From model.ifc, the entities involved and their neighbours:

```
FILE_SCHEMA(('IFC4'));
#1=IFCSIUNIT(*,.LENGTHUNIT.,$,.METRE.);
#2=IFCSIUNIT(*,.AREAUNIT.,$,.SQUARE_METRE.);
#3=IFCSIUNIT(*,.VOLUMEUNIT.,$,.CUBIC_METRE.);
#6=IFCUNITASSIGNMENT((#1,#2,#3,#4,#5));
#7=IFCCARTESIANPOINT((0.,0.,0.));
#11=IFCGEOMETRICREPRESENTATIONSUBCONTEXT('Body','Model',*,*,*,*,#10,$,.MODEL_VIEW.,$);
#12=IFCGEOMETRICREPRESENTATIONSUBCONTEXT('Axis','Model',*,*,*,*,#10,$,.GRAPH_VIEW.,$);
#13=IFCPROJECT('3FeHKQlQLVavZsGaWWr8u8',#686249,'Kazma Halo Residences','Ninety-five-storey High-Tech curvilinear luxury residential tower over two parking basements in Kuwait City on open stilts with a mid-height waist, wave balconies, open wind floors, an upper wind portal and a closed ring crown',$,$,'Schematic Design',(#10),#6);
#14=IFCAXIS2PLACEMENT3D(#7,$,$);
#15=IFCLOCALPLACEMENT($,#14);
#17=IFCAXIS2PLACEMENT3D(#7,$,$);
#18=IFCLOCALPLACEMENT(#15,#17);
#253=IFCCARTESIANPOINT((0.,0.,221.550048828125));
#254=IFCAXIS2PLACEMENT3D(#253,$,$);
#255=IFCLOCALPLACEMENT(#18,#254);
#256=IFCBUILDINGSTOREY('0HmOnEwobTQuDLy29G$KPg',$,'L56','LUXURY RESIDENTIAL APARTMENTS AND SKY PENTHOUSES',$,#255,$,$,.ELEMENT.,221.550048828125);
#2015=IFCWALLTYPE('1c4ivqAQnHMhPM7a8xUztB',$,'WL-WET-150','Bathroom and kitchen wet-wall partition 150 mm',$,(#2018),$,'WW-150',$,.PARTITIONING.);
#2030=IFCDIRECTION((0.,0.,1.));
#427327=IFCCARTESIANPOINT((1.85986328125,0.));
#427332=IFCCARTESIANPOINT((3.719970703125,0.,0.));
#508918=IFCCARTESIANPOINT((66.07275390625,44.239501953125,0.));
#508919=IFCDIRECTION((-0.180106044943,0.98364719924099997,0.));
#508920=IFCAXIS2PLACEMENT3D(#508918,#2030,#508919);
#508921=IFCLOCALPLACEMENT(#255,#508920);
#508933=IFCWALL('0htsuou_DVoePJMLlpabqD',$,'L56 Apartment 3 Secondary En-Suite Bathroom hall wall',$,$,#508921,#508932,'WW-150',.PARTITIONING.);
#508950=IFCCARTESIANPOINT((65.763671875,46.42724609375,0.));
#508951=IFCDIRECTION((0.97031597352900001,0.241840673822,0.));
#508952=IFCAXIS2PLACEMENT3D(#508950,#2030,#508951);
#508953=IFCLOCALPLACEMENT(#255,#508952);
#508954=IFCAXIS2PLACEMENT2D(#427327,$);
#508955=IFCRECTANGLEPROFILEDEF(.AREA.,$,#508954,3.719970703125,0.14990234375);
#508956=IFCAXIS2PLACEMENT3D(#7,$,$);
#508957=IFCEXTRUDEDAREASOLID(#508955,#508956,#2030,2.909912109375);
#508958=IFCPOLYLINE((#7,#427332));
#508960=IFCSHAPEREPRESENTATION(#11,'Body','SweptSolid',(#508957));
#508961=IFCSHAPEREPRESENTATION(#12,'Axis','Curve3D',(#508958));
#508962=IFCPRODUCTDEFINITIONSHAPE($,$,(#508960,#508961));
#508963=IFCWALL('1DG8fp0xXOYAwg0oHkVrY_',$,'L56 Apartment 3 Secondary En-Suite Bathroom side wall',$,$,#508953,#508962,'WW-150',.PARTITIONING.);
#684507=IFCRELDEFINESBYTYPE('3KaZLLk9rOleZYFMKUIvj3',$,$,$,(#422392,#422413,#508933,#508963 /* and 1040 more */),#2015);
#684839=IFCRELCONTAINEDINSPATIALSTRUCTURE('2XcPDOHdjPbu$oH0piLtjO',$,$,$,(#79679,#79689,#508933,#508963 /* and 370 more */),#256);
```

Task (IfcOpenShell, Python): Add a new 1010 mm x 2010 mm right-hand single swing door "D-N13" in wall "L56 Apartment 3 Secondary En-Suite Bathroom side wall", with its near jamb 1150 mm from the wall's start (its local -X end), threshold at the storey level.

```python
import numpy as np
import ifcopenshell
import ifcopenshell.api.feature
import ifcopenshell.api.geometry
import ifcopenshell.api.root
import ifcopenshell.api.spatial
import ifcopenshell.geom
import ifcopenshell.util.element
import ifcopenshell.util.placement
import ifcopenshell.util.representation
import ifcopenshell.util.shape
import ifcopenshell.util.unit

model = ifcopenshell.open("model.ifc")
unit_scale = ifcopenshell.util.unit.calculate_unit_scale(model)
settings = ifcopenshell.geom.settings()


def volume(element):
    """Net volume in cubic metres, openings subtracted."""
    shape = ifcopenshell.geom.create_shape(settings, element)
    return ifcopenshell.util.shape.get_volume(shape.geometry)


wall = model.by_id(508963)
storey = ifcopenshell.util.element.get_container(wall, ifc_class="IfcBuildingStorey")
context = ifcopenshell.util.representation.get_context(model, "Model", "Body", "MODEL_VIEW")
before = volume(wall)

width, height, from_end, sill = 1.01, 2.01, 1.15, 0.0  # metres

# The wall runs along its own X axis, and the end named is its -X end.
wall_shape = ifcopenshell.geom.create_shape(settings, wall)
x, y, z = ifcopenshell.util.shape.get_vertices(wall_shape.geometry).T
start = x.min() + from_end
face, thickness = float(y.min()), float(y.max() - y.min())
wall_matrix = ifcopenshell.util.placement.get_local_placement(wall.ObjectPlacement)
level = ifcopenshell.util.placement.get_local_placement(storey.ObjectPlacement)[2, 3]


def in_wall(x, y):
    """Placement at x, y metres in the wall's axes, at sill height."""
    matrix = wall_matrix.copy()
    matrix[:, 3] = wall_matrix @ np.array([x / unit_scale, y / unit_scale, 0.0, 1.0])
    matrix[2, 3] = level + sill / unit_scale
    return matrix


# Opening: a box that overshoots both wall faces by 50 mm.
opening = ifcopenshell.api.root.create_entity(model, ifc_class="IfcOpeningElement", predefined_type="OPENING")
box = ifcopenshell.api.geometry.add_wall_representation(
    model, context=context, length=width, height=height, thickness=thickness + 0.1
)
ifcopenshell.api.geometry.assign_representation(model, product=opening, representation=box)
ifcopenshell.api.geometry.edit_object_placement(model, product=opening, matrix=in_wall(start, face - 0.05), is_si=False)
ifcopenshell.api.feature.add_feature(model, feature=opening, element=wall)

door = ifcopenshell.api.root.create_entity(model, ifc_class="IfcDoor", name="D-N13", predefined_type="DOOR")
door.OverallWidth, door.OverallHeight = width / unit_scale, height / unit_scale
door.OperationType = "SINGLE_SWING_RIGHT"
body = ifcopenshell.api.geometry.add_door_representation(
    model,
    context=context,
    overall_width=door.OverallWidth,
    overall_height=door.OverallHeight,
    operation_type="SINGLE_SWING_RIGHT",
    lining_properties={"LiningDepth": thickness / unit_scale, "ThresholdDepth": thickness / unit_scale},
)
ifcopenshell.api.geometry.assign_representation(model, product=door, representation=body)
ifcopenshell.api.spatial.assign_container(model, products=[door], relating_structure=storey)
ifcopenshell.api.feature.add_filling(model, opening=opening, element=door)

# The lining spans the wall, so the door starts at the wall face.
ifcopenshell.api.geometry.edit_object_placement(model, product=door, matrix=in_wall(start, face), is_si=False)

after = volume(wall)

print(f"wall volume {before:.3f} -> {after:.3f} m3")

model.write("model-out.ifc")
```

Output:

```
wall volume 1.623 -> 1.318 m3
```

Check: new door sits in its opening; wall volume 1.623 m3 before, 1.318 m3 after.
